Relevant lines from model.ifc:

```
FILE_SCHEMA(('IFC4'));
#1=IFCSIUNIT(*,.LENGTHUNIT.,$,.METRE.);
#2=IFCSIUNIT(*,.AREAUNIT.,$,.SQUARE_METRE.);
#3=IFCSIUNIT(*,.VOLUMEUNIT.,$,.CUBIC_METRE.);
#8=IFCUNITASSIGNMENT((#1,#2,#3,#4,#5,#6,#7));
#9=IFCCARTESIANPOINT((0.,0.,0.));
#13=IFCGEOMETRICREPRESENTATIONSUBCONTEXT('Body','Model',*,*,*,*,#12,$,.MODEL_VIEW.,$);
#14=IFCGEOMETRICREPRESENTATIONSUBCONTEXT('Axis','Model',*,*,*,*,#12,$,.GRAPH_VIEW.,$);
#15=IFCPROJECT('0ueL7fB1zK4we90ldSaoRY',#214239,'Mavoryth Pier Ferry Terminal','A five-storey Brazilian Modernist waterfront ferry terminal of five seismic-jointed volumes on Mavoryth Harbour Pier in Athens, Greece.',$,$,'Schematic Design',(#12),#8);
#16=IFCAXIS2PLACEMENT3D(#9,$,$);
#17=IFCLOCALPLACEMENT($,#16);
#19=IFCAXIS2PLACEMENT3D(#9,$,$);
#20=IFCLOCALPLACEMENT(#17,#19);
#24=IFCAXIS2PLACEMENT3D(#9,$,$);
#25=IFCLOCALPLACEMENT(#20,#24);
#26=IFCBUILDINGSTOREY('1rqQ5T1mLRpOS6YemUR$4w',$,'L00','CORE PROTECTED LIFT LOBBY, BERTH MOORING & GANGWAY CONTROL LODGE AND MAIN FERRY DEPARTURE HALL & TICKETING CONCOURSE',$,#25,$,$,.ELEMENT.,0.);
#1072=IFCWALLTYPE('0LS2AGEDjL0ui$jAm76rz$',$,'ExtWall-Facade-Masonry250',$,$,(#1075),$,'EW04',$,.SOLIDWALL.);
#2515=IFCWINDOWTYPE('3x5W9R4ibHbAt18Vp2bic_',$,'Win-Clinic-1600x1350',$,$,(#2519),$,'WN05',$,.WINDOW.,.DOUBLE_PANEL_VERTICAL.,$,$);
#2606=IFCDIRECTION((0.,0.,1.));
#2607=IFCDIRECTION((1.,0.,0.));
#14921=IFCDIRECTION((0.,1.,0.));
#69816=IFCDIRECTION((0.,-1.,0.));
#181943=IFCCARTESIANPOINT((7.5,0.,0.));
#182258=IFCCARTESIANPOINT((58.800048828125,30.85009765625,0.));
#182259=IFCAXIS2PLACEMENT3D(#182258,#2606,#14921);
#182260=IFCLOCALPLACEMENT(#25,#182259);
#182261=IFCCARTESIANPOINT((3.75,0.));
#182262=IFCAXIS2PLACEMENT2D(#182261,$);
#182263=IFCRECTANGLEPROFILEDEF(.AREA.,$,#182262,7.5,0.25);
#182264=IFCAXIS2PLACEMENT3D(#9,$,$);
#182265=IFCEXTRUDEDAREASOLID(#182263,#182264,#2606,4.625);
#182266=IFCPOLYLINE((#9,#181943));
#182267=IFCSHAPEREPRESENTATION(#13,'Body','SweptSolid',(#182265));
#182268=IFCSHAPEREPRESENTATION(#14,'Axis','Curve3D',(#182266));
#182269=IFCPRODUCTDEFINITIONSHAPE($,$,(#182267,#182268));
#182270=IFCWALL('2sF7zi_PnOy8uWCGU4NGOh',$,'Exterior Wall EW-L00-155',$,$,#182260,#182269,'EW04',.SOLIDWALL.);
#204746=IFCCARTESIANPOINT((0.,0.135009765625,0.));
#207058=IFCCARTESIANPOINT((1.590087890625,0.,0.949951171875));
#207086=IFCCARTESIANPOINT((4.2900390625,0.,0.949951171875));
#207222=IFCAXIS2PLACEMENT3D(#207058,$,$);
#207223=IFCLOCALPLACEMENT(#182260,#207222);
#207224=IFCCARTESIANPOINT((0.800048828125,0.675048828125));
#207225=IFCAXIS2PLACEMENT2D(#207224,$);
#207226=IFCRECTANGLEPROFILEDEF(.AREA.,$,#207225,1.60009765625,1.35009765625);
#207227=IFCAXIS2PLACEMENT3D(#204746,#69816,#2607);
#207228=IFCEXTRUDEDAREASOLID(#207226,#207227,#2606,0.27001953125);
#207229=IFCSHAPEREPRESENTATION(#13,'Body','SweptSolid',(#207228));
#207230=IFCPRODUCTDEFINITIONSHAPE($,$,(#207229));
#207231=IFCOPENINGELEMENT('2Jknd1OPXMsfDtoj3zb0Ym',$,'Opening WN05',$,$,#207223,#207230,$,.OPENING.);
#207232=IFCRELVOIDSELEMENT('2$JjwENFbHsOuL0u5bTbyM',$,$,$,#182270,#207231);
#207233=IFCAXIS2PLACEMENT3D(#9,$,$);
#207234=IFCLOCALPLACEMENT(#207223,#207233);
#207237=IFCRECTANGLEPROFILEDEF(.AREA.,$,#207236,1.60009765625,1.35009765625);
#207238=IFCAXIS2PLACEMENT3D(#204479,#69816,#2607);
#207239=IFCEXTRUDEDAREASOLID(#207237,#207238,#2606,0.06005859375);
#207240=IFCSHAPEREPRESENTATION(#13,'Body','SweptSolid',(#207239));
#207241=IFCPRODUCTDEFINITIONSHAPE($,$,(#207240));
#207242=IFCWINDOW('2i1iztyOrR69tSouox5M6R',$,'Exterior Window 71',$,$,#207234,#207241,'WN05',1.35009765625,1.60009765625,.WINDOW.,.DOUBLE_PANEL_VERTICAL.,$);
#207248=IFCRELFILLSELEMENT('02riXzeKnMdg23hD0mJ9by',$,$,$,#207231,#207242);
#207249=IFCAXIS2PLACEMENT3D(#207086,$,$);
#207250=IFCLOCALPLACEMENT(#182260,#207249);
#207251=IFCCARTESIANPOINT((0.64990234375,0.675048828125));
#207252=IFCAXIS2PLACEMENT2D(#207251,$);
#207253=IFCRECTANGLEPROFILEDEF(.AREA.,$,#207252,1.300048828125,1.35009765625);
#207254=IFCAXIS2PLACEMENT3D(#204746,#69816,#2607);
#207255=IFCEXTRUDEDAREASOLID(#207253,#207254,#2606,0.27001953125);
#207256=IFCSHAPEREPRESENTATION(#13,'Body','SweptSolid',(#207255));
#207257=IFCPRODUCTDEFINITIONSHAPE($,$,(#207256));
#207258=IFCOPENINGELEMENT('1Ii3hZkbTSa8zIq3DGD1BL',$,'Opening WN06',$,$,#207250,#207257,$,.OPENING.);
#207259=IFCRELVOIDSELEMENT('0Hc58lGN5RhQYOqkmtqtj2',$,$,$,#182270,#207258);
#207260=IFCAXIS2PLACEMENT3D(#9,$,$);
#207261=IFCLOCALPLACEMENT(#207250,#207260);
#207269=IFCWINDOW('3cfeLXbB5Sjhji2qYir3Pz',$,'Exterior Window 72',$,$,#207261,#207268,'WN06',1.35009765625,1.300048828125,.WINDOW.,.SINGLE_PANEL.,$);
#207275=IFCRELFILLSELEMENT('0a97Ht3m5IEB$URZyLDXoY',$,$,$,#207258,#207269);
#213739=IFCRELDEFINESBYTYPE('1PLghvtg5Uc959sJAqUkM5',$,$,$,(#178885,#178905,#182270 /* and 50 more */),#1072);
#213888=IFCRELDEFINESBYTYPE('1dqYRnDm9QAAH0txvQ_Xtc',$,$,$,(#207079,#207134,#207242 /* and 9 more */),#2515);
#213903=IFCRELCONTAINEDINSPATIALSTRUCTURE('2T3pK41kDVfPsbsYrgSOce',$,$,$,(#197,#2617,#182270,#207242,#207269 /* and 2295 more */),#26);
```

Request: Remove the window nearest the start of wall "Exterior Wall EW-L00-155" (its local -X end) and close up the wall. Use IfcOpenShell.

```python
import ifcopenshell
import ifcopenshell.api.feature
import ifcopenshell.api.root
import ifcopenshell.geom
import ifcopenshell.util.shape

model = ifcopenshell.open("model.ifc")
settings = ifcopenshell.geom.settings()


def volume(element):
    """Net volume in cubic metres, openings subtracted."""
    shape = ifcopenshell.geom.create_shape(settings, element)
    return ifcopenshell.util.shape.get_volume(shape.geometry)


window = model.by_guid("2i1iztyOrR69tSouox5M6R")
opening = window.FillsVoids[0].RelatingOpeningElement
wall = opening.VoidsElements[0].RelatingBuildingElement
before = volume(wall)

ifcopenshell.api.root.remove_product(model, product=window)
ifcopenshell.api.feature.remove_feature(model, feature=opening)

after = volume(wall)

print(f"wall volume {before:.3f} -> {after:.3f} m3")

model.write("model_rev.ifc")
```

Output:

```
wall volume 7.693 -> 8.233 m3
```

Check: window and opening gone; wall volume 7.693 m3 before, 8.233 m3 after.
